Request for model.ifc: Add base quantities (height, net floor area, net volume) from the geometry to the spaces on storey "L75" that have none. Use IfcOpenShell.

First a look at what the model holds.

```python
import ifcopenshell
import ifcopenshell.util.element
import ifcopenshell.util.unit

model = ifcopenshell.open("model.ifc")
print(model.schema)
for unit_type in ("LENGTHUNIT", "AREAUNIT", "VOLUMEUNIT"):
    print(unit_type, ifcopenshell.util.unit.calculate_unit_scale(model, unit_type))
storey = next(s for s in model.by_type("IfcBuildingStorey") if s.Name == "L75")
spaces = [e for e in ifcopenshell.util.element.get_decomposition(storey) if e.is_a("IfcSpace")]
for e in sorted(spaces, key=lambda e: e.id()):
    print(e.id(), e.is_a(), e.Name, list(ifcopenshell.util.element.get_psets(e, qtos_only=True)), sep=" | ")
```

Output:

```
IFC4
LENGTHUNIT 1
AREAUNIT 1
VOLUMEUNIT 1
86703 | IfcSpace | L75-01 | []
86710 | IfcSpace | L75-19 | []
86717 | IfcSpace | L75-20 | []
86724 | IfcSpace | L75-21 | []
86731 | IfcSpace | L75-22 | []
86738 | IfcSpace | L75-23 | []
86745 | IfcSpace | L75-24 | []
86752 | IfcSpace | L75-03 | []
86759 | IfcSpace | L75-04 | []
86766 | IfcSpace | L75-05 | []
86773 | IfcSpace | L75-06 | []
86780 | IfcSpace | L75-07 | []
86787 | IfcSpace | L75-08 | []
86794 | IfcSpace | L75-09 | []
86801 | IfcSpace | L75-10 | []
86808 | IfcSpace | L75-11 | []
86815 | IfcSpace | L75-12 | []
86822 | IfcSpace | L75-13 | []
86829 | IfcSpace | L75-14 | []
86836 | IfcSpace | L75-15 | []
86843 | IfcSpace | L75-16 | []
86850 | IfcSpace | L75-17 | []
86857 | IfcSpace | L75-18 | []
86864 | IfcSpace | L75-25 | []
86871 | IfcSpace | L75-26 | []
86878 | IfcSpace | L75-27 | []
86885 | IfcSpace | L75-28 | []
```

```python
import ifcopenshell
import ifcopenshell.api.pset
import ifcopenshell.geom
import ifcopenshell.util.element
import ifcopenshell.util.shape
import ifcopenshell.util.unit

model = ifcopenshell.open("model.ifc")
unit_scale = ifcopenshell.util.unit.calculate_unit_scale(model)
area_scale = ifcopenshell.util.unit.calculate_unit_scale(model, "AREAUNIT")
volume_scale = ifcopenshell.util.unit.calculate_unit_scale(model, "VOLUMEUNIT")
settings = ifcopenshell.geom.settings()

storey = next(s for s in model.by_type("IfcBuildingStorey") if s.Name == "L75")
spaces = [e for e in ifcopenshell.util.element.get_decomposition(storey) if e.is_a("IfcSpace")]

for e in sorted(spaces, key=lambda e: e.id()):
    if ifcopenshell.util.element.get_psets(e, qtos_only=True, should_inherit=False):
        continue
    # Geometry comes back in metres, in the element's own axes.
    shape = ifcopenshell.geom.create_shape(settings, e)
    values = {
        "Height": ifcopenshell.util.shape.get_z(shape.geometry) / unit_scale,
        "NetFloorArea": ifcopenshell.util.shape.get_footprint_area(shape.geometry) / area_scale,
        "NetVolume": ifcopenshell.util.shape.get_volume(shape.geometry) / volume_scale,
    }
    qto = ifcopenshell.api.pset.add_qto(model, product=e, name="Qto_SpaceBaseQuantities")
    ifcopenshell.api.pset.edit_qto(model, qto=qto, properties=values)
    print(e.id(), {k: round(v, 3) for k, v in values.items()})

model.write("model_rev.ifc")
```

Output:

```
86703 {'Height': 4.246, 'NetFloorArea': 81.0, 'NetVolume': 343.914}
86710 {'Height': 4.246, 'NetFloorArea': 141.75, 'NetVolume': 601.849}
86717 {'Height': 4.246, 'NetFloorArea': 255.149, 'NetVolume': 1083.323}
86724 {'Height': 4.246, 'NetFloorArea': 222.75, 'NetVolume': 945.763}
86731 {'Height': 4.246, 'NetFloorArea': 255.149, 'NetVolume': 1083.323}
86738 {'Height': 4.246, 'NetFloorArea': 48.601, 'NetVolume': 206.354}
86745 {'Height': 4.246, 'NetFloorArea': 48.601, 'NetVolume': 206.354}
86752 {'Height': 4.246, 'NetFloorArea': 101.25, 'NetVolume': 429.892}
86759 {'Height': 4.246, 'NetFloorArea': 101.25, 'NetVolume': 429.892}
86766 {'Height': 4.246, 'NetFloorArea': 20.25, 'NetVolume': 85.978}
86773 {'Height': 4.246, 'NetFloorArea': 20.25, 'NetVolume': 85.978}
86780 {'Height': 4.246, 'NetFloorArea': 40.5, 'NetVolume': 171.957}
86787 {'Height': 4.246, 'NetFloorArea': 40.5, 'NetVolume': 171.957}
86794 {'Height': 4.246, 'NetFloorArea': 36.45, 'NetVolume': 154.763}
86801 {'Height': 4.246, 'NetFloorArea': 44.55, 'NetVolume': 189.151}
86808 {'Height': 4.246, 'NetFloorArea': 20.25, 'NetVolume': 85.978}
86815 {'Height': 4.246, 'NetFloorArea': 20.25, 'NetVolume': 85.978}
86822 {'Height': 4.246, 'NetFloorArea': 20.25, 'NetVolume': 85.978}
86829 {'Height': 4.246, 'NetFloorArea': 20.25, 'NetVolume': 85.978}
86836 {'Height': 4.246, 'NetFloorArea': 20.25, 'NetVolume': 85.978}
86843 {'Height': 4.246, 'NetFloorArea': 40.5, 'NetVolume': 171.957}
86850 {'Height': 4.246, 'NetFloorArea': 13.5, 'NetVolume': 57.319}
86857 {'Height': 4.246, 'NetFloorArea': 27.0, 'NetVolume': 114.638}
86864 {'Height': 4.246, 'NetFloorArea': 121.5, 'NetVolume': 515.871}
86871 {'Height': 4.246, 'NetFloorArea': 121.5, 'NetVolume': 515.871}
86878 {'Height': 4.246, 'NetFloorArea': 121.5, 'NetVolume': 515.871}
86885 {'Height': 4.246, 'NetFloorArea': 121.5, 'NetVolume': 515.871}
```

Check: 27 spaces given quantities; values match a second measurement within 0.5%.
